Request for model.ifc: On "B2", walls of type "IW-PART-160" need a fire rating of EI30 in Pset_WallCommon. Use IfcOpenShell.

First a look at what the model holds.

```python
import ifcopenshell
import ifcopenshell.util.element

model = ifcopenshell.open("model.ifc")
print(model.schema)
storey = next(s for s in model.by_type("IfcBuildingStorey") if s.Name == "B2")
walls = [e for e in ifcopenshell.util.element.get_decomposition(storey) if e.is_a("IfcWall")]
seen = {}
for e in walls:
    element_type = ifcopenshell.util.element.get_type(e)
    key = (element_type.Name if element_type != e and element_type else None, ifcopenshell.util.element.get_pset(e, "Pset_WallCommon", "FireRating"))
    seen[key] = seen.get(key, 0) + 1
for (name, value), count in sorted(seen.items(), key=str):
    print(count, "x", name, "|", value)
```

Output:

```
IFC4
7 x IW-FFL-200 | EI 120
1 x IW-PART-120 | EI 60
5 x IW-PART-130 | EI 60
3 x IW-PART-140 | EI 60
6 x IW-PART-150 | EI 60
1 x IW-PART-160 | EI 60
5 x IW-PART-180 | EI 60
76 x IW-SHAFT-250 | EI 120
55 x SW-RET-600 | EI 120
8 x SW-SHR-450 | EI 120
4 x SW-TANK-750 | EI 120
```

```python
import ifcopenshell
import ifcopenshell.api.pset
import ifcopenshell.util.element

model = ifcopenshell.open("model.ifc")

storey = next(s for s in model.by_type("IfcBuildingStorey") if s.Name == "B2")
walls = [e for e in ifcopenshell.util.element.get_decomposition(storey) if e.is_a("IfcWall")]

count = 0
for e in walls:
    element_type = ifcopenshell.util.element.get_type(e)
    if element_type in (None, e) or element_type.Name != "IW-PART-160":
        continue
    # add_pset returns the element's existing set when there is one.
    pset = ifcopenshell.api.pset.add_pset(model, product=e, name="Pset_WallCommon")
    ifcopenshell.api.pset.edit_pset(model, pset=pset, properties={"FireRating": "EI30"})
    count += 1

print(count, "walls updated")

model.write("model-out.ifc")
```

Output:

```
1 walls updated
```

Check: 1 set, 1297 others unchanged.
